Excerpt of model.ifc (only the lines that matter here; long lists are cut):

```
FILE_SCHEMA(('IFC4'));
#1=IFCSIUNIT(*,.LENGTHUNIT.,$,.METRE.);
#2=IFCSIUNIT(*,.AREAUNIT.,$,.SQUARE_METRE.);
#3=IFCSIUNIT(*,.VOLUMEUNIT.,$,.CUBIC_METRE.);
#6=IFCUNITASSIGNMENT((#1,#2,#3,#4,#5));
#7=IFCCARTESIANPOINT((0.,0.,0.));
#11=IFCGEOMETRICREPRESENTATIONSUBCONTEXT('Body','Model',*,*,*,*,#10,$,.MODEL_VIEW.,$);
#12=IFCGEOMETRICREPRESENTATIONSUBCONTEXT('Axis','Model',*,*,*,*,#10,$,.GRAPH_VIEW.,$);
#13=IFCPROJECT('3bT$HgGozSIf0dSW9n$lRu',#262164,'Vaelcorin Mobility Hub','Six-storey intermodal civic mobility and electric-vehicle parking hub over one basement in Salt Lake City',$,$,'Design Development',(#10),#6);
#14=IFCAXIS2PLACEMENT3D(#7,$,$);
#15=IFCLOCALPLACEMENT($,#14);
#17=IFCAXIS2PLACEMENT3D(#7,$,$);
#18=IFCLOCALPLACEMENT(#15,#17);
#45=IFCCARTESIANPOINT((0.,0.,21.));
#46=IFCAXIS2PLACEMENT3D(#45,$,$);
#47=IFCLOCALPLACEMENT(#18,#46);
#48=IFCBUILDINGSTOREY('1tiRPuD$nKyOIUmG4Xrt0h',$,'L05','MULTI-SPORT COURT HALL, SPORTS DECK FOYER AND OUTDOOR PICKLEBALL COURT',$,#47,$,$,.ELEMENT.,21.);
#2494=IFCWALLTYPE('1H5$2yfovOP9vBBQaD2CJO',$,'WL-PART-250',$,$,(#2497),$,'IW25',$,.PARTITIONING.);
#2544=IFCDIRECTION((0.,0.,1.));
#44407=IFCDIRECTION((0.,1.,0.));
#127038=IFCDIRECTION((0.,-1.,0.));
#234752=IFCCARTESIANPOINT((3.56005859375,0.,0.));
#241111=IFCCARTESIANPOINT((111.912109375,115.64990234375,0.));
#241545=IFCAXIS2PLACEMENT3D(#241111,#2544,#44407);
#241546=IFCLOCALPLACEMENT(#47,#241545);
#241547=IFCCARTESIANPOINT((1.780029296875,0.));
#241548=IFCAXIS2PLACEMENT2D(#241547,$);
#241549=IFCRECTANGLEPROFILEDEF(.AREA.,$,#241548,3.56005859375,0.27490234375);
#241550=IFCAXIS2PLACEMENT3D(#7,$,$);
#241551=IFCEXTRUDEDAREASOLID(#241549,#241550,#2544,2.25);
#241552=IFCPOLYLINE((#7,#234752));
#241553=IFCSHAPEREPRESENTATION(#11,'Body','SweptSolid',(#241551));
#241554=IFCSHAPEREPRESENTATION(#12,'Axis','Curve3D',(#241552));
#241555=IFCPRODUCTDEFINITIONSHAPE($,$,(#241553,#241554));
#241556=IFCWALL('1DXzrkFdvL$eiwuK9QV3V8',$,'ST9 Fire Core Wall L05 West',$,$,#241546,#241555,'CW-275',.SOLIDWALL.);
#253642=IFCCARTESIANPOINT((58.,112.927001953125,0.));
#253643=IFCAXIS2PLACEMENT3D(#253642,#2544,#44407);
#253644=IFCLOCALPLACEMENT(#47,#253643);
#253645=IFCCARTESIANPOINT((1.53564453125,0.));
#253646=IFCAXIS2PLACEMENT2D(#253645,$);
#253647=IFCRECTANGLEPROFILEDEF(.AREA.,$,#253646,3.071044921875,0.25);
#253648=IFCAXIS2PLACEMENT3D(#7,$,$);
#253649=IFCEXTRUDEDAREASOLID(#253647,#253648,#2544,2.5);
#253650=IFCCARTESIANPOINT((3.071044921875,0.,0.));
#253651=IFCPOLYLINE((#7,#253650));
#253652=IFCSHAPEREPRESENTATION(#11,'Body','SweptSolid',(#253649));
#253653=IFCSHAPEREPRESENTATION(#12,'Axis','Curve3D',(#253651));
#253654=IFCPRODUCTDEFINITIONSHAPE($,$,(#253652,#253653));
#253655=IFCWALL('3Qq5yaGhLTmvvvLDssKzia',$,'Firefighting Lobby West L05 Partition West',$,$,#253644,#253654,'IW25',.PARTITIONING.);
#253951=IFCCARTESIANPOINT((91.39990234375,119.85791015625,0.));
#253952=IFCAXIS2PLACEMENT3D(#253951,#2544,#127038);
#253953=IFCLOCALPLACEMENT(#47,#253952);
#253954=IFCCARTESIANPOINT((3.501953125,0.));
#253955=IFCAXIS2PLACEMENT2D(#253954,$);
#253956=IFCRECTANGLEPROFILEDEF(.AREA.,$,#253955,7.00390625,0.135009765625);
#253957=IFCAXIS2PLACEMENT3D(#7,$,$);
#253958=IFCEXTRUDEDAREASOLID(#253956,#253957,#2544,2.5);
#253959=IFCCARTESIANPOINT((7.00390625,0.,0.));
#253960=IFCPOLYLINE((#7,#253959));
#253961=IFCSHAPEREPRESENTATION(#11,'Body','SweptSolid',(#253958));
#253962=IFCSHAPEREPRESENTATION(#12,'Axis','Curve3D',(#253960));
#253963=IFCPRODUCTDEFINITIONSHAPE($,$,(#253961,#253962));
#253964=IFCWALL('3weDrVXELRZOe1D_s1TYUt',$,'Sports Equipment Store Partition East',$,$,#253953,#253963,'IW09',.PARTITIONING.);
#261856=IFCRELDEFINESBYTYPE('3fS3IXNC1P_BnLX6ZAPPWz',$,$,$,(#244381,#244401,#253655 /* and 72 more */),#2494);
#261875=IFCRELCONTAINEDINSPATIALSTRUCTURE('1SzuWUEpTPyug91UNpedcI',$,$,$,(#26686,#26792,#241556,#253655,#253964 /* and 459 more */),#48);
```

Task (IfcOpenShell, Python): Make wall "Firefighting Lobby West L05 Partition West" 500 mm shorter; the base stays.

```python
import ifcopenshell
import ifcopenshell.geom
import ifcopenshell.util.representation
import ifcopenshell.util.shape
import ifcopenshell.util.unit

model = ifcopenshell.open("model.ifc")
unit_scale = ifcopenshell.util.unit.calculate_unit_scale(model)
settings = ifcopenshell.geom.settings()


def volume(element):
    """Net volume in cubic metres, openings subtracted."""
    shape = ifcopenshell.geom.create_shape(settings, element)
    return ifcopenshell.util.shape.get_volume(shape.geometry)


wall = model.by_id(253655)
before = volume(wall)

body = ifcopenshell.util.representation.get_representation(wall, "Model", "Body")
solid = body.Items[0]
old_height = solid.Depth
solid.Depth -= 0.5 / unit_scale
after = volume(wall)

print(f"height {old_height:g} -> {solid.Depth:g}, volume {before:.3f} -> {after:.3f} m3")

model.write("model_edited.ifc")
```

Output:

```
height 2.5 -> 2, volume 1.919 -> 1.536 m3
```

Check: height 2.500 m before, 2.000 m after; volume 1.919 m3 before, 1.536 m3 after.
